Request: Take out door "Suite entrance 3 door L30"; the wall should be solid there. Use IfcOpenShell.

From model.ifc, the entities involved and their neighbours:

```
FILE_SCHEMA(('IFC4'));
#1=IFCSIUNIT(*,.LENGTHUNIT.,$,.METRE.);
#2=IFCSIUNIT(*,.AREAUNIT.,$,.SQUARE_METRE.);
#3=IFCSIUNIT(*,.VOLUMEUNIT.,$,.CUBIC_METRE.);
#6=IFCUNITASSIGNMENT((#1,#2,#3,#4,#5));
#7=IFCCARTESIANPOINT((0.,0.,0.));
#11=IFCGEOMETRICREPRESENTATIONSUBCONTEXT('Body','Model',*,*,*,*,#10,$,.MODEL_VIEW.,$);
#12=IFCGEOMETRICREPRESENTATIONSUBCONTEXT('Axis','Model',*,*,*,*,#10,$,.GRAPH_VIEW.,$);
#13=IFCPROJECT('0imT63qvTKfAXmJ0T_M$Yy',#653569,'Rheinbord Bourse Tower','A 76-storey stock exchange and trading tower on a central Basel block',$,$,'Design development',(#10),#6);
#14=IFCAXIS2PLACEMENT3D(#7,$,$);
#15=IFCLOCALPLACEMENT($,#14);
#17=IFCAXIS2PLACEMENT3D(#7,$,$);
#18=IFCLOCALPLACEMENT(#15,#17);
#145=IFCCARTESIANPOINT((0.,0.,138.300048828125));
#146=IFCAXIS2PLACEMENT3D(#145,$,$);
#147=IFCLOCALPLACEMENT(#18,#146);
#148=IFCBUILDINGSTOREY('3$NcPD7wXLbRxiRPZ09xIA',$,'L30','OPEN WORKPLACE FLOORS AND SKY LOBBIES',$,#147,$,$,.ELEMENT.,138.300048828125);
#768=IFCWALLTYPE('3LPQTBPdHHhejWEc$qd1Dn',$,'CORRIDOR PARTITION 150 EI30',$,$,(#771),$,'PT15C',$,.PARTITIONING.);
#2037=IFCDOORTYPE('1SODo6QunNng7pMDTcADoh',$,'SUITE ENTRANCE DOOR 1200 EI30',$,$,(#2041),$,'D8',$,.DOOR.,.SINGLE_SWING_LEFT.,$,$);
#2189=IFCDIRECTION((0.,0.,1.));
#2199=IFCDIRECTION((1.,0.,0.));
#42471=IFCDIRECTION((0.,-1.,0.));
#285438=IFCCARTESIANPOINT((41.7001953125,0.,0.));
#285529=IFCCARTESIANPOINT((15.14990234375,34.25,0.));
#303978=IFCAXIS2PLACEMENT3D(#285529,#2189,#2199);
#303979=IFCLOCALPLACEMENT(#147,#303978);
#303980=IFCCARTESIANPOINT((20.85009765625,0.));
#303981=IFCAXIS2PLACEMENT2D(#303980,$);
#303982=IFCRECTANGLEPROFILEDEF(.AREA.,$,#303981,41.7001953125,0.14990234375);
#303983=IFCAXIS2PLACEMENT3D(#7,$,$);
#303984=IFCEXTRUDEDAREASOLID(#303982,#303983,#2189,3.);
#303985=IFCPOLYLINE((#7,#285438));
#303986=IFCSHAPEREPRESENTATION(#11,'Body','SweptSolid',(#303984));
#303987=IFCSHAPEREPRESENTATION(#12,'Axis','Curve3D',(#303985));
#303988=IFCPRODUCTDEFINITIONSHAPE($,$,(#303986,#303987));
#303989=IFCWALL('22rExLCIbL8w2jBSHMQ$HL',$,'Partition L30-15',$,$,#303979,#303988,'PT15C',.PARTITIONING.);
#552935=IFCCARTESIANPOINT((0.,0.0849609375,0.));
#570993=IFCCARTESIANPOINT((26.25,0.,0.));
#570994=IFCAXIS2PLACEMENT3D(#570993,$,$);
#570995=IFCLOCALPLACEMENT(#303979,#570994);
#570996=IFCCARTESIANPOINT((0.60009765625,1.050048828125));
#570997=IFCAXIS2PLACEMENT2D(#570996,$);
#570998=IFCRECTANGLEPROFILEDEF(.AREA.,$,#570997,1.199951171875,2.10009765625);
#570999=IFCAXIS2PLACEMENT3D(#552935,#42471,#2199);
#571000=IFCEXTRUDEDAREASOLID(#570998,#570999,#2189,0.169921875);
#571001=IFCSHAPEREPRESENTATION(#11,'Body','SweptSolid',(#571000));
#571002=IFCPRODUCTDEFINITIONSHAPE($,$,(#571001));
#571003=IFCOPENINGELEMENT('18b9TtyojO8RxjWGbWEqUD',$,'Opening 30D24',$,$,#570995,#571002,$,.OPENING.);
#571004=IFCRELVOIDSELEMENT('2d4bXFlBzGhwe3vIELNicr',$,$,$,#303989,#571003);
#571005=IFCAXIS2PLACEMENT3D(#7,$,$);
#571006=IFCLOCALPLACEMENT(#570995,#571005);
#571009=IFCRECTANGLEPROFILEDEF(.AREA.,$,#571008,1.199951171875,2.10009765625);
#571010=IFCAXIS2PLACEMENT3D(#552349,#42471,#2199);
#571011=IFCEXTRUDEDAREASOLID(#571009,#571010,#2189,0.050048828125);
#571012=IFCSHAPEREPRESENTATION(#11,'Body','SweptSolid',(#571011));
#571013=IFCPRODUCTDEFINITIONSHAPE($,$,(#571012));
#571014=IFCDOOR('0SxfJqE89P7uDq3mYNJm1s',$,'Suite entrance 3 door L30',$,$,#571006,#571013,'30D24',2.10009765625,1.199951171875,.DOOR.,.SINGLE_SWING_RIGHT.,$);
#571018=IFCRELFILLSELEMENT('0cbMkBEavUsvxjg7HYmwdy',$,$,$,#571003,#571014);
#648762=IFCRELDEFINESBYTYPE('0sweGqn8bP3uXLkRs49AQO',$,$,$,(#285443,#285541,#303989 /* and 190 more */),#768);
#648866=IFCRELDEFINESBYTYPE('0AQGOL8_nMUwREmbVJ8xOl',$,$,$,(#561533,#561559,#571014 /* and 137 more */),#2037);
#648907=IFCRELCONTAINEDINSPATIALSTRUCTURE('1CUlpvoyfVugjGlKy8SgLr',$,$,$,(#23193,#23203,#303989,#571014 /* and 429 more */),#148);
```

```python
import ifcopenshell
import ifcopenshell.api.feature
import ifcopenshell.api.root
import ifcopenshell.geom
import ifcopenshell.util.shape

model = ifcopenshell.open("model.ifc")
settings = ifcopenshell.geom.settings()


def volume(element):
    """Net volume in cubic metres, openings subtracted."""
    shape = ifcopenshell.geom.create_shape(settings, element)
    return ifcopenshell.util.shape.get_volume(shape.geometry)


door = model.by_guid("0SxfJqE89P7uDq3mYNJm1s")
opening = door.FillsVoids[0].RelatingOpeningElement
wall = opening.VoidsElements[0].RelatingBuildingElement
before = volume(wall)

ifcopenshell.api.root.remove_product(model, product=door)
ifcopenshell.api.feature.remove_feature(model, feature=opening)

after = volume(wall)

print(f"wall volume {before:.3f} -> {after:.3f} m3")

model.write("model-out.ifc")
```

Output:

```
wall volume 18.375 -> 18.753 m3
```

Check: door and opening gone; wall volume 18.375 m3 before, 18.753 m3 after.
